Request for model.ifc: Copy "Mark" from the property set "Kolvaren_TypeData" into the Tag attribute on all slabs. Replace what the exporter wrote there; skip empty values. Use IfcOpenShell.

First a look at what the model holds.

```python
import ifcopenshell
import ifcopenshell.util.element

model = ifcopenshell.open("model.ifc")
print(model.schema)
slabs = model.by_type("IfcSlab")
print(len(slabs), "slabs")
for e in slabs[:8]:
    source = ifcopenshell.util.element.get_pset(e, "Kolvaren_TypeData", "Mark")
    target = e.Tag
    print(e.id(), repr(source), repr(target), sep=" | ")
```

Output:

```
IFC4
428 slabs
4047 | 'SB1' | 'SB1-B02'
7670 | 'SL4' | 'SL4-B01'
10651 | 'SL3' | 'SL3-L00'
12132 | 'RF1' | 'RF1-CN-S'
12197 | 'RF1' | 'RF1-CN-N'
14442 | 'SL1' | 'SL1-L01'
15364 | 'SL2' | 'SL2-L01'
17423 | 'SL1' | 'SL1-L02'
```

```python
import ifcopenshell
import ifcopenshell.util.element

model = ifcopenshell.open("model.ifc")

count = 0
for e in model.by_type("IfcSlab"):
    value = ifcopenshell.util.element.get_pset(e, "Kolvaren_TypeData", "Mark")
    current = e.Tag
    if not value or not value.strip() or current == value:
        continue
    e.Tag = value
    count += 1

print(count, "slabs updated")

model.write("model_v2.ifc")
```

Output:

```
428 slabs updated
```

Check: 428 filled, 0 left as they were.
